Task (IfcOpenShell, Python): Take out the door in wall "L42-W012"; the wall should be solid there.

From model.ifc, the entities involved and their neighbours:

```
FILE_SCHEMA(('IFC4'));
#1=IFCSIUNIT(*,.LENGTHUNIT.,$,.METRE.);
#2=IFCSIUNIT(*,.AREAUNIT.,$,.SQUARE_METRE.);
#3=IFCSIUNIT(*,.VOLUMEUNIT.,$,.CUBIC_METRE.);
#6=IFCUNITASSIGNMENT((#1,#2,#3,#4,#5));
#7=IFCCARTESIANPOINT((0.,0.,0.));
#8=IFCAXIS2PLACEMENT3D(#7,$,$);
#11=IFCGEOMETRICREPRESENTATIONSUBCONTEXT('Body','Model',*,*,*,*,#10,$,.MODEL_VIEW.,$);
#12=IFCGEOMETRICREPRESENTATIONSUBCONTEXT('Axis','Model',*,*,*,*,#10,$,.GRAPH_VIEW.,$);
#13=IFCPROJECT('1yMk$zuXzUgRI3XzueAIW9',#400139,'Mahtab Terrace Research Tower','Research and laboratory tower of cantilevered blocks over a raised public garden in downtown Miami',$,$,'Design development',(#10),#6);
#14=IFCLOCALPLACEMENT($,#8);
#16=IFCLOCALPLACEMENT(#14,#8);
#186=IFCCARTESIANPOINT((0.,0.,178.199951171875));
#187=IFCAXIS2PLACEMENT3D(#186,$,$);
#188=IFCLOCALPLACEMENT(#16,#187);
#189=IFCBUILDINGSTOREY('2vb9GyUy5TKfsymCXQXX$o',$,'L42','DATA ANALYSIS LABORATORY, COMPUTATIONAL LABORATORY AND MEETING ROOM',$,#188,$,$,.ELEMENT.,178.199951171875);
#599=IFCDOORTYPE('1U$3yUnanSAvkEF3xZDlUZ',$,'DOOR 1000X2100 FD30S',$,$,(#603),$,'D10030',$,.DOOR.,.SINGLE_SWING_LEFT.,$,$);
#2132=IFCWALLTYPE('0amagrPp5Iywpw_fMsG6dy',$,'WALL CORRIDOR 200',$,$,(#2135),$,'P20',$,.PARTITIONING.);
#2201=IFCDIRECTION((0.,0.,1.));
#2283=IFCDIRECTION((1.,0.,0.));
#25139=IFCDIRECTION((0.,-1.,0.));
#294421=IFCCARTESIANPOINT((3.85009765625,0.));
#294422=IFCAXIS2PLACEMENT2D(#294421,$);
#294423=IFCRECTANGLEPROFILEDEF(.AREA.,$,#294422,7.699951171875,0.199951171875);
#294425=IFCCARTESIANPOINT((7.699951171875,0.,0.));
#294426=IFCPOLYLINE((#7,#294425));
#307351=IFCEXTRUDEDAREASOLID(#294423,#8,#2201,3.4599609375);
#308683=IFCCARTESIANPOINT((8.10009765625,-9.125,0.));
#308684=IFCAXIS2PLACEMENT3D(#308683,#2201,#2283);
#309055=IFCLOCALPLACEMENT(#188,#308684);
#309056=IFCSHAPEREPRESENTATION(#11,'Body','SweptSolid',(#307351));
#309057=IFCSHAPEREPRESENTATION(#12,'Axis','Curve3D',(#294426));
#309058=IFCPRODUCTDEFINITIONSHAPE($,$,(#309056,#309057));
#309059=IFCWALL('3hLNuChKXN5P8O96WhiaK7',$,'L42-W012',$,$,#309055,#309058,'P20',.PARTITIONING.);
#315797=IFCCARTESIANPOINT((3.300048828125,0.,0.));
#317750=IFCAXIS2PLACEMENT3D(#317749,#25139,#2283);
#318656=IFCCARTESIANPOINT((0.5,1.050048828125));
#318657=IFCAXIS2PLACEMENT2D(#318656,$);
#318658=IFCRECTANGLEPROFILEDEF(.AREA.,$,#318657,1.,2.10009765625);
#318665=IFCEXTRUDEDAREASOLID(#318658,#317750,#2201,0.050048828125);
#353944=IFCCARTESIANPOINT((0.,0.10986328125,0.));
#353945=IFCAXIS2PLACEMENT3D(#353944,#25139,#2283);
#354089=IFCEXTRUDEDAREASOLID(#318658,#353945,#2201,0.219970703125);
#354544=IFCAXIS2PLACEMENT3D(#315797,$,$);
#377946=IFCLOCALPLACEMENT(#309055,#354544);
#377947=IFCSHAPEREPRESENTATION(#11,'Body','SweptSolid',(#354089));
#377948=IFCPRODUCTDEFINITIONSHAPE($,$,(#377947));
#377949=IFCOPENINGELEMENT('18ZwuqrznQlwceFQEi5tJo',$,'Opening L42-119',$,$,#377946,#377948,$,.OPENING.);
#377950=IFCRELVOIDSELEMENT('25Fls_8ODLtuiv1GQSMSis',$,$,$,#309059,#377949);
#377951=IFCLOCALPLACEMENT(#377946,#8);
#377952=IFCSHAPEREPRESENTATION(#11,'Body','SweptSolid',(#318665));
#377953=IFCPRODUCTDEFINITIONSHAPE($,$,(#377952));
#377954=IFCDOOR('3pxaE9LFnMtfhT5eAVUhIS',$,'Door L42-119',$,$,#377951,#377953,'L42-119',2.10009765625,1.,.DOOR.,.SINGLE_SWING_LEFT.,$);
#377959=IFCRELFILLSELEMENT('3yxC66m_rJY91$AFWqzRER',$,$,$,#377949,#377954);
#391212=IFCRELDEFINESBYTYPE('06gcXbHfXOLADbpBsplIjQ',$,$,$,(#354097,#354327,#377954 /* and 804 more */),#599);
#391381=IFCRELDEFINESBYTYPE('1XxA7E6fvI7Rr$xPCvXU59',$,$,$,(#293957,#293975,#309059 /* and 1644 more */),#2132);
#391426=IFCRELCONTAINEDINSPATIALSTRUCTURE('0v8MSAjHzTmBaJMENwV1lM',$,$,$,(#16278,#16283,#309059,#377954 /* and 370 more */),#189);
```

```python
import ifcopenshell
import ifcopenshell.api.feature
import ifcopenshell.api.root
import ifcopenshell.geom
import ifcopenshell.util.shape

model = ifcopenshell.open("model.ifc")
settings = ifcopenshell.geom.settings()


def volume(element):
    """Net volume in cubic metres, openings subtracted."""
    shape = ifcopenshell.geom.create_shape(settings, element)
    return ifcopenshell.util.shape.get_volume(shape.geometry)


door = model.by_guid("3pxaE9LFnMtfhT5eAVUhIS")
opening = door.FillsVoids[0].RelatingOpeningElement
wall = opening.VoidsElements[0].RelatingBuildingElement
before = volume(wall)

ifcopenshell.api.root.remove_product(model, product=door)
ifcopenshell.api.feature.remove_feature(model, feature=opening)

after = volume(wall)

print(f"wall volume {before:.3f} -> {after:.3f} m3")

model.write("model_rev.ifc")
```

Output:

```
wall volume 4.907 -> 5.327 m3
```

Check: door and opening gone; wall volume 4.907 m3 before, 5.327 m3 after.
